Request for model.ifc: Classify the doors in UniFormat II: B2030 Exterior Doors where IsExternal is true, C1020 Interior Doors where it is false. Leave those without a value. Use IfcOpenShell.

First a look at what the model holds.

```python
import ifcopenshell
import ifcopenshell.util.element

model = ifcopenshell.open("model.ifc")
print(model.schema)
print("classifications:", [c.Name for c in model.by_type("IfcClassification")])
values = [ifcopenshell.util.element.get_pset(e, "Pset_DoorCommon", "IsExternal") for e in model.by_type("IfcDoor")]
for value in (True, False, None):
    print("IsExternal", value, values.count(value))
```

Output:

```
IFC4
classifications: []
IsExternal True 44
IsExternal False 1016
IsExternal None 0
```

```python
import ifcopenshell
import ifcopenshell.api.classification
import ifcopenshell.util.element

model = ifcopenshell.open("model.ifc")

system = ifcopenshell.api.classification.add_classification(model, classification="UniFormat II")

doors = model.by_type("IfcDoor")
external = {e: ifcopenshell.util.element.get_pset(e, "Pset_DoorCommon", "IsExternal") for e in doors}
for flag, code, name in ((True, "B2030", "Exterior Doors"), (False, "C1020", "Interior Doors")):
    products = [e for e in doors if external[e] is flag]
    ifcopenshell.api.classification.add_reference(
        model, products=products, classification=system, identification=code, name=name
    )
    print(code, len(products))

model.write("model_v2.ifc")
```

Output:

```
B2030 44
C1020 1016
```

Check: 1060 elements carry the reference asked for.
